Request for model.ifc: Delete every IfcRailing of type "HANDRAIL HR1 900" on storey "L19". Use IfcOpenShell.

First a look at what the model holds.

```python
import ifcopenshell
import ifcopenshell.util.element

model = ifcopenshell.open("model.ifc")
print(model.schema)
storey = next(s for s in model.by_type("IfcBuildingStorey") if s.Name == "L19")
railings = [e for e in ifcopenshell.util.element.get_decomposition(storey) if e.is_a("IfcRailing")]
seen = {}
for e in railings:
    element_type = ifcopenshell.util.element.get_type(e)
    name = element_type.Name if element_type not in (None, e) else None
    seen[name] = seen.get(name, 0) + 1
for name, count in sorted(seen.items(), key=str):
    print(count, "x", name)
```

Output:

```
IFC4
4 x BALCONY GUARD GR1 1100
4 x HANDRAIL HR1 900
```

```python
import ifcopenshell
import ifcopenshell.api.root
import ifcopenshell.util.element

model = ifcopenshell.open("model.ifc")

storey = next(s for s in model.by_type("IfcBuildingStorey") if s.Name == "L19")
railings = [e for e in ifcopenshell.util.element.get_decomposition(storey) if e.is_a("IfcRailing")]
targets = [e for e in railings if (t := ifcopenshell.util.element.get_type(e)) not in (None, e) and t.Name == "HANDRAIL HR1 900"]

for e in targets:
    ifcopenshell.api.root.remove_product(model, product=e)
print(len(targets), "removed")

model.write("model_updated.ifc")
```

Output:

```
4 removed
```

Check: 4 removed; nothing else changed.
